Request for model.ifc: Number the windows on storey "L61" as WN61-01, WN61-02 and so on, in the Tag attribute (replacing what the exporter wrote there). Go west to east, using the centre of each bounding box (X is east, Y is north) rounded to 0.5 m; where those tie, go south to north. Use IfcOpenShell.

First a look at what the model holds.

```python
import ifcopenshell
import ifcopenshell.util.element
import ifcopenshell.util.placement

model = ifcopenshell.open("model.ifc")
print(model.schema)
storey = next(s for s in model.by_type("IfcBuildingStorey") if s.Name == "L61")
windows = [e for e in ifcopenshell.util.element.get_decomposition(storey) if e.is_a("IfcWindow")]
for e in sorted(windows, key=lambda e: e.id()):
    origin = ifcopenshell.util.placement.get_local_placement(e.ObjectPlacement)[:3, 3]
    print(e.id(), e.Tag, e.Name, origin.round(2) + 0.0, sep=" | ")
```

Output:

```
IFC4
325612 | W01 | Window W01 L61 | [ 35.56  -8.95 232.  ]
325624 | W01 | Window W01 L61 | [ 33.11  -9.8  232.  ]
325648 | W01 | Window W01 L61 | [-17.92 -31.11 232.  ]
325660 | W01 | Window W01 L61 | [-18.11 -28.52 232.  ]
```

```python
import ifcopenshell
import ifcopenshell.geom
import ifcopenshell.util.element
import ifcopenshell.util.shape

model = ifcopenshell.open("model.ifc")
settings = ifcopenshell.geom.settings()
settings.set("use-world-coords", True)


def centre(element):
    shape = ifcopenshell.geom.create_shape(settings, element)
    return ifcopenshell.util.shape.get_bbox_centroid(shape.geometry)


storey = next(s for s in model.by_type("IfcBuildingStorey") if s.Name == "L61")
windows = [e for e in ifcopenshell.util.element.get_decomposition(storey) if e.is_a("IfcWindow")]

# Insertion points can sit at a corner or the storey origin, so sort by the geometry (in metres).
centres = {e: centre(e) for e in windows}
windows.sort(key=lambda e: (round(centres[e][0] / 0.5), centres[e][1]))

for i, e in enumerate(windows, start=1):
    number = f"WN61-{i:02d}"
    e.Tag = number
    print(e.id(), number)

model.write("model_rev.ifc")
```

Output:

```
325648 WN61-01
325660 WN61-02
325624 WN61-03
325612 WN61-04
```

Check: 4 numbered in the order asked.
